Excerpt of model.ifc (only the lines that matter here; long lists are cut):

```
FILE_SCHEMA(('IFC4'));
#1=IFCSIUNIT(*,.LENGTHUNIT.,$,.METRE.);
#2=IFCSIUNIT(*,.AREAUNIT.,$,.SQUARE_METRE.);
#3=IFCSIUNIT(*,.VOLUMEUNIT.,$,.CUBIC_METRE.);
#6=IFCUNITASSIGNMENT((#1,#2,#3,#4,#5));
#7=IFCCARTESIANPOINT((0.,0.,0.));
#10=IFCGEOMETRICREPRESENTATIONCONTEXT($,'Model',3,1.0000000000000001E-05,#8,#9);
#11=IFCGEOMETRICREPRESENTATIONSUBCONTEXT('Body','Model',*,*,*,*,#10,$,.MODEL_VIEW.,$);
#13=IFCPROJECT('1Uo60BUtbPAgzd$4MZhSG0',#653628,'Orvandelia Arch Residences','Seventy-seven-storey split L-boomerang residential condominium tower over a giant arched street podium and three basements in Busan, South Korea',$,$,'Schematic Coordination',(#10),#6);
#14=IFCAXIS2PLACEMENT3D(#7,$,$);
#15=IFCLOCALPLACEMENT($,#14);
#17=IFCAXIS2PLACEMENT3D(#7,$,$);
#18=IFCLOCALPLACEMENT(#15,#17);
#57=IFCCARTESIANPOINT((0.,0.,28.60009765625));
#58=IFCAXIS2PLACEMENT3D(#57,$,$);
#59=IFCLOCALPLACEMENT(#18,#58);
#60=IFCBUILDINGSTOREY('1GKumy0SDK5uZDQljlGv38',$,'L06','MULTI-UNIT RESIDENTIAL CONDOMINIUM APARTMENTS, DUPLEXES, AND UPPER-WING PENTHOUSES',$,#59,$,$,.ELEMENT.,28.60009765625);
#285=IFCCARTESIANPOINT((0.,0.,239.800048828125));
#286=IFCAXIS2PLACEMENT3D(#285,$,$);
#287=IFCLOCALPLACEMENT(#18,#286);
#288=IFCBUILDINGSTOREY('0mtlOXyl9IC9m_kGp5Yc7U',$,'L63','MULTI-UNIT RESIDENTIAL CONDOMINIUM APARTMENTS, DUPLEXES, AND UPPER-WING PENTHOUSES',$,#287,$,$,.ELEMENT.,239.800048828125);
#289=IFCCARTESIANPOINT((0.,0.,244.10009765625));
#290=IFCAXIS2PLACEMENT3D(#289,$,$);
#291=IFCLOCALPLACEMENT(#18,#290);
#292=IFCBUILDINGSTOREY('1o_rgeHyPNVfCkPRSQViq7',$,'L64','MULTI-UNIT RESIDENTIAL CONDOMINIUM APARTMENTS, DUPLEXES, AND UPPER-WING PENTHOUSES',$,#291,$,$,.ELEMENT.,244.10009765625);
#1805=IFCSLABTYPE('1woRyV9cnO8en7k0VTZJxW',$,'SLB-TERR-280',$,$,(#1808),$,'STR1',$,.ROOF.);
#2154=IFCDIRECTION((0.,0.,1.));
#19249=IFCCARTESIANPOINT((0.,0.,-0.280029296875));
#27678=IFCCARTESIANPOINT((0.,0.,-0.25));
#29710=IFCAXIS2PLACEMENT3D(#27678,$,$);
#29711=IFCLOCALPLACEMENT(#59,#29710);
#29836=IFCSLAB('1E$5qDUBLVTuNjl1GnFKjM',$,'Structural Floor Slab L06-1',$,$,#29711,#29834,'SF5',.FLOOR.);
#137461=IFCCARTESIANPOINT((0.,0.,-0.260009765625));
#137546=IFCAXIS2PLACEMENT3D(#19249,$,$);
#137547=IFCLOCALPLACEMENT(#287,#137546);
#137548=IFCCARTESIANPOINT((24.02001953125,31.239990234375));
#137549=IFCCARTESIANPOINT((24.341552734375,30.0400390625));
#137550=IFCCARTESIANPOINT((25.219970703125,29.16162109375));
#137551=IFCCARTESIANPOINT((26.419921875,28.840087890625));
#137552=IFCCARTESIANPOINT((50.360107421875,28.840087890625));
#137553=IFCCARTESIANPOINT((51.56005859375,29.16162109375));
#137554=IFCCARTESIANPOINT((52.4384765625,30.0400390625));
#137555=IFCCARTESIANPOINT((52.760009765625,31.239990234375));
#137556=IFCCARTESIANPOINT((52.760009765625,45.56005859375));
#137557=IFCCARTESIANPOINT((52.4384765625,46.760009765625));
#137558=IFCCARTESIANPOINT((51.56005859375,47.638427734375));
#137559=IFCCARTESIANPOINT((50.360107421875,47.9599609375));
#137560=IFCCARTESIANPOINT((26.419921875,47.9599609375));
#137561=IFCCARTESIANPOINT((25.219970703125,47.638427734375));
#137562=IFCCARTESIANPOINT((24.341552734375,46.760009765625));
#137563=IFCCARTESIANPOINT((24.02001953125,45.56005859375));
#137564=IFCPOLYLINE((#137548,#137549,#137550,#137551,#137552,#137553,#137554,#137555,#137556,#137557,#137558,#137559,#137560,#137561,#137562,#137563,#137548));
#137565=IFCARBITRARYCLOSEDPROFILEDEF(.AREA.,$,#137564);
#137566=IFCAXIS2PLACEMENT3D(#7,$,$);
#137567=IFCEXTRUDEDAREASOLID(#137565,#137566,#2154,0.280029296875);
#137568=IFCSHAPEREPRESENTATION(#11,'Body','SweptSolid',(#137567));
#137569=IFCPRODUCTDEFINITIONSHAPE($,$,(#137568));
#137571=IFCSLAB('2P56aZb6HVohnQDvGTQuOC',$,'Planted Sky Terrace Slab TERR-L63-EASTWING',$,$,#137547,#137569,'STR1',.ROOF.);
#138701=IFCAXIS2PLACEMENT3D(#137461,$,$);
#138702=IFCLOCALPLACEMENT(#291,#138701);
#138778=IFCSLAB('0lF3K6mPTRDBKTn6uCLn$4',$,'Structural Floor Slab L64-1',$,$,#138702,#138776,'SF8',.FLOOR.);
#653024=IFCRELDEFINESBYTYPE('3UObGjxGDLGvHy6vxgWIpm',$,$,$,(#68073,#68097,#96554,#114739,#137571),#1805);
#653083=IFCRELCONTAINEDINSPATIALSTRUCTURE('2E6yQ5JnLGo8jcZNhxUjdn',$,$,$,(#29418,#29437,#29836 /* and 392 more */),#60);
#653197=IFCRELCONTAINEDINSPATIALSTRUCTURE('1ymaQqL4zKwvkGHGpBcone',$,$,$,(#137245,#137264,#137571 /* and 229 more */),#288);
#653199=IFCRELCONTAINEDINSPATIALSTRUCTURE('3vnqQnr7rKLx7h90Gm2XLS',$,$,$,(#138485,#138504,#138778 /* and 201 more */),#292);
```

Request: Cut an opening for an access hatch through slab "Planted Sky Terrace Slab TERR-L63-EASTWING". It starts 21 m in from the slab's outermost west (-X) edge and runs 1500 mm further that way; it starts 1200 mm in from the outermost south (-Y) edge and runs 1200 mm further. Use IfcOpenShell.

```python
import numpy as np
import ifcopenshell
import ifcopenshell.api.feature
import ifcopenshell.api.geometry
import ifcopenshell.api.root
import ifcopenshell.geom
import ifcopenshell.util.placement
import ifcopenshell.util.representation
import ifcopenshell.util.shape
import ifcopenshell.util.unit

model = ifcopenshell.open("model.ifc")
unit_scale = ifcopenshell.util.unit.calculate_unit_scale(model)
settings = ifcopenshell.geom.settings()


def volume(element):
    """Net volume in cubic metres, openings subtracted."""
    shape = ifcopenshell.geom.create_shape(settings, element)
    return ifcopenshell.util.shape.get_volume(shape.geometry)


slab = model.by_guid("2P56aZb6HVohnQDvGTQuOC")
before = volume(slab)

# Extent in the slab's own axes, in metres. The edges named are its -X and -Y sides.
slab_shape = ifcopenshell.geom.create_shape(settings, slab)
vertices = ifcopenshell.util.shape.get_vertices(slab_shape.geometry)
x_min, y_min, bottom = vertices.min(axis=0)
top = vertices[:, 2].max()

opening = ifcopenshell.api.root.create_entity(model, ifc_class="IfcOpeningElement", name="Access hatch opening", predefined_type="OPENING")
context = ifcopenshell.util.representation.get_context(model, "Model", "Body", "MODEL_VIEW")
width, depth = 1.5, 1.2
outline = [(0.0, 0.0), (width, 0.0), (width, depth), (0.0, depth), (0.0, 0.0)]
# Overshoot both faces by 50 mm so the cut is clean.
shape = ifcopenshell.api.geometry.add_slab_representation(
    model, context=context, depth=top - bottom + 0.1, polyline=outline
)
ifcopenshell.api.geometry.assign_representation(model, product=opening, representation=shape)

matrix = ifcopenshell.util.placement.get_local_placement(slab.ObjectPlacement)
matrix[:, 3] = matrix @ np.append(np.array([x_min + 21, y_min + 1.2, bottom - 0.05]) / unit_scale, 1.0)
ifcopenshell.api.geometry.edit_object_placement(model, product=opening, matrix=matrix, is_si=False)
ifcopenshell.api.feature.add_feature(model, feature=opening, element=slab)

after = volume(slab)

print(f"slab volume {before:.3f} -> {after:.3f} m3")

model.write("model_edited.ifc")
```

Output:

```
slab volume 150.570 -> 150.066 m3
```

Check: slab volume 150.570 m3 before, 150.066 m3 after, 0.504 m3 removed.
